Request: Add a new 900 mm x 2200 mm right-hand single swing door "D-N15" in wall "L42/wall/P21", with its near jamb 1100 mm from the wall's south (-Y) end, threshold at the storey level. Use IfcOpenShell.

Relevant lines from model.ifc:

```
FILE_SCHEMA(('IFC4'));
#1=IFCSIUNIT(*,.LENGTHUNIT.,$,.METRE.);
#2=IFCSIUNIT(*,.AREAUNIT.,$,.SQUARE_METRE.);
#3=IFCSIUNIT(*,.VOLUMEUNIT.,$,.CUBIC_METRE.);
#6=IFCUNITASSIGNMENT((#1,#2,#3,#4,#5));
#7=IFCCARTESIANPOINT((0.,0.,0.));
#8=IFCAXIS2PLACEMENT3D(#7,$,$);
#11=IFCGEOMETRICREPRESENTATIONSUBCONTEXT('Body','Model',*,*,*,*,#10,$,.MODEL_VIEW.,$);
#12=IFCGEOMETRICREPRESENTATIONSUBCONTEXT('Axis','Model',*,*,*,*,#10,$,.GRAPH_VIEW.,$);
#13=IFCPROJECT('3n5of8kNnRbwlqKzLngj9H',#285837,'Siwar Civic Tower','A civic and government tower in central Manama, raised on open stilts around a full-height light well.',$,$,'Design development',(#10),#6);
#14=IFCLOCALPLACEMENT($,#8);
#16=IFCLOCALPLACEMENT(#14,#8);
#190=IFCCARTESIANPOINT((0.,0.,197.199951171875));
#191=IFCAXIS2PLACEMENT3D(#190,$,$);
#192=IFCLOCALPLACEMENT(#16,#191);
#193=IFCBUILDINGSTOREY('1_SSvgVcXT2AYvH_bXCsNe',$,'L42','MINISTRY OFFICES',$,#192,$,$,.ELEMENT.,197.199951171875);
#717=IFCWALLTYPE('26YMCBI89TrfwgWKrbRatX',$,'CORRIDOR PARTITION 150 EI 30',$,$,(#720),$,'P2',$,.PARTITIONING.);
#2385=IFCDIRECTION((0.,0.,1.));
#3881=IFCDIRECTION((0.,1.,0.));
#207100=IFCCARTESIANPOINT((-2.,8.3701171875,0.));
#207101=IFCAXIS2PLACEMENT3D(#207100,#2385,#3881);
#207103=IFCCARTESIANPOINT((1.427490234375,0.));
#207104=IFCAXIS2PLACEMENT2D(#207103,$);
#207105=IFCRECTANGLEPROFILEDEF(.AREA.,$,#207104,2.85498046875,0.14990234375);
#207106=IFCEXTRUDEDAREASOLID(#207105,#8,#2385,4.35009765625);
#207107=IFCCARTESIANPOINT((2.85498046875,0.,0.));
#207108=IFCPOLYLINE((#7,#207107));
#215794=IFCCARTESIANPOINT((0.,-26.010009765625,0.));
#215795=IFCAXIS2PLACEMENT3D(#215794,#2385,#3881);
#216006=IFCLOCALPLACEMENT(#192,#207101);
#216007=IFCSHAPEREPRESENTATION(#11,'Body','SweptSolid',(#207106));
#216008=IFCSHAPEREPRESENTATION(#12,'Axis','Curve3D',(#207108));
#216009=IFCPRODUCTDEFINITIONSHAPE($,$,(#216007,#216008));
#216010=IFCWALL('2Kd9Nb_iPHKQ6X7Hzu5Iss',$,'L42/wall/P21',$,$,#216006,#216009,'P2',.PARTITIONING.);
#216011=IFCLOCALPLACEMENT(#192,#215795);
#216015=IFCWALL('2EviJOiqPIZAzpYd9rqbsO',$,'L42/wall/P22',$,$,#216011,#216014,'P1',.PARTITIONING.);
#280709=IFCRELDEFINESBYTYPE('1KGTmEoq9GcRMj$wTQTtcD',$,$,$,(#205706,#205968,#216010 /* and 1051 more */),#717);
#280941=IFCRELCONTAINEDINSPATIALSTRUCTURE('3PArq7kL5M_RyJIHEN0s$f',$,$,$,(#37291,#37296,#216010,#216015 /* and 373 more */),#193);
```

```python
import numpy as np
import ifcopenshell
import ifcopenshell.api.feature
import ifcopenshell.api.geometry
import ifcopenshell.api.root
import ifcopenshell.api.spatial
import ifcopenshell.geom
import ifcopenshell.util.element
import ifcopenshell.util.placement
import ifcopenshell.util.representation
import ifcopenshell.util.shape
import ifcopenshell.util.unit

model = ifcopenshell.open("model.ifc")
unit_scale = ifcopenshell.util.unit.calculate_unit_scale(model)
settings = ifcopenshell.geom.settings()


def volume(element):
    """Net volume in cubic metres, openings subtracted."""
    shape = ifcopenshell.geom.create_shape(settings, element)
    return ifcopenshell.util.shape.get_volume(shape.geometry)


wall = model.by_id(216010)
storey = ifcopenshell.util.element.get_container(wall, ifc_class="IfcBuildingStorey")
context = ifcopenshell.util.representation.get_context(model, "Model", "Body", "MODEL_VIEW")
before = volume(wall)

width, height, from_end, sill = 0.9, 2.2, 1.1, 0.0  # metres

# The wall runs along its own X axis, and the end named is its -X end.
wall_shape = ifcopenshell.geom.create_shape(settings, wall)
x, y, z = ifcopenshell.util.shape.get_vertices(wall_shape.geometry).T
start = x.min() + from_end
face, thickness = float(y.min()), float(y.max() - y.min())
wall_matrix = ifcopenshell.util.placement.get_local_placement(wall.ObjectPlacement)
level = ifcopenshell.util.placement.get_local_placement(storey.ObjectPlacement)[2, 3]


def in_wall(x, y):
    """Placement at x, y metres in the wall's axes, at sill height."""
    matrix = wall_matrix.copy()
    matrix[:, 3] = wall_matrix @ np.array([x / unit_scale, y / unit_scale, 0.0, 1.0])
    matrix[2, 3] = level + sill / unit_scale
    return matrix


# Opening: a box that overshoots both wall faces by 50 mm.
opening = ifcopenshell.api.root.create_entity(model, ifc_class="IfcOpeningElement", predefined_type="OPENING")
box = ifcopenshell.api.geometry.add_wall_representation(
    model, context=context, length=width, height=height, thickness=thickness + 0.1
)
ifcopenshell.api.geometry.assign_representation(model, product=opening, representation=box)
ifcopenshell.api.geometry.edit_object_placement(model, product=opening, matrix=in_wall(start, face - 0.05), is_si=False)
ifcopenshell.api.feature.add_feature(model, feature=opening, element=wall)

door = ifcopenshell.api.root.create_entity(model, ifc_class="IfcDoor", name="D-N15", predefined_type="DOOR")
door.OverallWidth, door.OverallHeight = width / unit_scale, height / unit_scale
door.OperationType = "SINGLE_SWING_RIGHT"
body = ifcopenshell.api.geometry.add_door_representation(
    model,
    context=context,
    overall_width=door.OverallWidth,
    overall_height=door.OverallHeight,
    operation_type="SINGLE_SWING_RIGHT",
    lining_properties={"LiningDepth": thickness / unit_scale, "ThresholdDepth": thickness / unit_scale},
)
ifcopenshell.api.geometry.assign_representation(model, product=door, representation=body)
ifcopenshell.api.spatial.assign_container(model, products=[door], relating_structure=storey)
ifcopenshell.api.feature.add_filling(model, opening=opening, element=door)

# The lining spans the wall, so the door starts at the wall face.
ifcopenshell.api.geometry.edit_object_placement(model, product=door, matrix=in_wall(start, face), is_si=False)

after = volume(wall)

print(f"wall volume {before:.3f} -> {after:.3f} m3")

model.write("model_updated.ifc")
```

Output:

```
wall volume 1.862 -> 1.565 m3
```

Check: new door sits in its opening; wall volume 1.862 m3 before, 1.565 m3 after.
